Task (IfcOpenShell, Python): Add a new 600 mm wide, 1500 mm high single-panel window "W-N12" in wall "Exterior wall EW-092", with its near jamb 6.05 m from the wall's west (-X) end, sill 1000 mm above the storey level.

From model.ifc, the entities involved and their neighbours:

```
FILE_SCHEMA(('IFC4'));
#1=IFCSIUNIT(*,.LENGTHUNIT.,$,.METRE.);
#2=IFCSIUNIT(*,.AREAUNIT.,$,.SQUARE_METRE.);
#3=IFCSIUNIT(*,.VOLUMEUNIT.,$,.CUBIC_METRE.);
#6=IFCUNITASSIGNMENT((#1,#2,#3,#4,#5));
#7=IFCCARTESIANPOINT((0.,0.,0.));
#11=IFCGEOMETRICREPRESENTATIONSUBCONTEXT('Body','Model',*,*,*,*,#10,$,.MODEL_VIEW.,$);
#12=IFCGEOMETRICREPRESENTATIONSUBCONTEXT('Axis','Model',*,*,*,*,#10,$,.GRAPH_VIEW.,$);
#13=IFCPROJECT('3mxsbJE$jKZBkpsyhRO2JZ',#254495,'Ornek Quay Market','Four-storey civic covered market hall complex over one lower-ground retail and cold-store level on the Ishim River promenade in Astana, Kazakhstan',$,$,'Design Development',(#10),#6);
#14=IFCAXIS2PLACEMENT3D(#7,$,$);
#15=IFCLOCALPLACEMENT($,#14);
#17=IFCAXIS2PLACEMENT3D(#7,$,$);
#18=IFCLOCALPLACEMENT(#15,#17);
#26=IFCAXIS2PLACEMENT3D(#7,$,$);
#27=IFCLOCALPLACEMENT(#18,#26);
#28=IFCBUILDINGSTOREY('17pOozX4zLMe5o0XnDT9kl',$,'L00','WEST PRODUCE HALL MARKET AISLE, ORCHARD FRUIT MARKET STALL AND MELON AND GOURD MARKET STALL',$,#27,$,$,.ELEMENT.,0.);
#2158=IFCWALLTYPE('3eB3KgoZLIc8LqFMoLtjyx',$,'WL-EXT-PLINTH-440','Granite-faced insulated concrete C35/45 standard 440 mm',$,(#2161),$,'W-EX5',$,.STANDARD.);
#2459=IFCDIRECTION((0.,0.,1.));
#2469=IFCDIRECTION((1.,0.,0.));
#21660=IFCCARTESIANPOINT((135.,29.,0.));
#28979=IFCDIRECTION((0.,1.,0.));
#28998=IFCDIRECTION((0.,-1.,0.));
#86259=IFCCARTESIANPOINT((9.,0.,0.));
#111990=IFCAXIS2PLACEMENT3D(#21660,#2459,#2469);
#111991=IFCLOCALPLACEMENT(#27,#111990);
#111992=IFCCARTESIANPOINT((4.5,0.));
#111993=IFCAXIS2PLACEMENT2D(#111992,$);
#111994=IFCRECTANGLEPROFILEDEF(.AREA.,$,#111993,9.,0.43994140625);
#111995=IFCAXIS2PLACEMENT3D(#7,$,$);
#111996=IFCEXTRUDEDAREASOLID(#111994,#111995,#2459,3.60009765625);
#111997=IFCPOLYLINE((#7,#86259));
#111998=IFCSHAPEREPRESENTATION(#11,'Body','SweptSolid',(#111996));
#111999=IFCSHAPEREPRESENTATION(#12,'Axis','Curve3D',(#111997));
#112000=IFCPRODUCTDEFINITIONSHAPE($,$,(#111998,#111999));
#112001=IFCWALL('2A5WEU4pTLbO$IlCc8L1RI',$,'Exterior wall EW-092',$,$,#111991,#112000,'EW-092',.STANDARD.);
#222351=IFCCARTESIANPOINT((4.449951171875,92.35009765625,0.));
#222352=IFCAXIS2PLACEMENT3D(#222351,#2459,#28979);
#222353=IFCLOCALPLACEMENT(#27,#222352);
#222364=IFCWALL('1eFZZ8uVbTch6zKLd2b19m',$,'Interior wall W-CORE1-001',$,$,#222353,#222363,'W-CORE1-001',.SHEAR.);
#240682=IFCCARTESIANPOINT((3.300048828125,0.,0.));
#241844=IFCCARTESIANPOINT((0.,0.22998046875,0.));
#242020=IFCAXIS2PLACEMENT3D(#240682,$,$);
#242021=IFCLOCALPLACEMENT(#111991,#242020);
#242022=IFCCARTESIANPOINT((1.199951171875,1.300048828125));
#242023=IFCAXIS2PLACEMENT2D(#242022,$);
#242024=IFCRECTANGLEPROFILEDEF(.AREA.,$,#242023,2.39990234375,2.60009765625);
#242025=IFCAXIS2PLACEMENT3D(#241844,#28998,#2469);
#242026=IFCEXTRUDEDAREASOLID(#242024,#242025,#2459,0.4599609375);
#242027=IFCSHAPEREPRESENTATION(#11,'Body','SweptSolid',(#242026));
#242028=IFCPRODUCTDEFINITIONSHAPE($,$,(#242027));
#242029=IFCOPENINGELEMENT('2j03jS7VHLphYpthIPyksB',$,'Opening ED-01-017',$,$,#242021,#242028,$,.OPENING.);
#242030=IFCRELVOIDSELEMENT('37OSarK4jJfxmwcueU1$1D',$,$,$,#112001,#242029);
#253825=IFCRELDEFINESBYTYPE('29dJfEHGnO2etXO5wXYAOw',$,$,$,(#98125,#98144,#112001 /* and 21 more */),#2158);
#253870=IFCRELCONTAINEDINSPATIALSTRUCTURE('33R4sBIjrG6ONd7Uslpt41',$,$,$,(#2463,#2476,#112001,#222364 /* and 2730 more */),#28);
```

```python
import numpy as np
import ifcopenshell
import ifcopenshell.api.feature
import ifcopenshell.api.geometry
import ifcopenshell.api.root
import ifcopenshell.api.spatial
import ifcopenshell.geom
import ifcopenshell.util.element
import ifcopenshell.util.placement
import ifcopenshell.util.representation
import ifcopenshell.util.shape
import ifcopenshell.util.unit

model = ifcopenshell.open("model.ifc")
unit_scale = ifcopenshell.util.unit.calculate_unit_scale(model)
settings = ifcopenshell.geom.settings()


def volume(element):
    """Net volume in cubic metres, openings subtracted."""
    shape = ifcopenshell.geom.create_shape(settings, element)
    return ifcopenshell.util.shape.get_volume(shape.geometry)


wall = model.by_guid("2A5WEU4pTLbO$IlCc8L1RI")
storey = ifcopenshell.util.element.get_container(wall, ifc_class="IfcBuildingStorey")
context = ifcopenshell.util.representation.get_context(model, "Model", "Body", "MODEL_VIEW")
before = volume(wall)

width, height, from_end, sill = 0.6, 1.5, 6.05, 1  # metres

# The wall runs along its own X axis, and the end named is its -X end.
wall_shape = ifcopenshell.geom.create_shape(settings, wall)
x, y, z = ifcopenshell.util.shape.get_vertices(wall_shape.geometry).T
start = x.min() + from_end
face, thickness = float(y.min()), float(y.max() - y.min())
wall_matrix = ifcopenshell.util.placement.get_local_placement(wall.ObjectPlacement)
level = ifcopenshell.util.placement.get_local_placement(storey.ObjectPlacement)[2, 3]


def in_wall(x, y):
    """Placement at x, y metres in the wall's axes, at sill height."""
    matrix = wall_matrix.copy()
    matrix[:, 3] = wall_matrix @ np.array([x / unit_scale, y / unit_scale, 0.0, 1.0])
    matrix[2, 3] = level + sill / unit_scale
    return matrix


# Opening: a box that overshoots both wall faces by 50 mm.
opening = ifcopenshell.api.root.create_entity(model, ifc_class="IfcOpeningElement", predefined_type="OPENING")
box = ifcopenshell.api.geometry.add_wall_representation(
    model, context=context, length=width, height=height, thickness=thickness + 0.1
)
ifcopenshell.api.geometry.assign_representation(model, product=opening, representation=box)
ifcopenshell.api.geometry.edit_object_placement(model, product=opening, matrix=in_wall(start, face - 0.05), is_si=False)
ifcopenshell.api.feature.add_feature(model, feature=opening, element=wall)

window = ifcopenshell.api.root.create_entity(model, ifc_class="IfcWindow", name="W-N12", predefined_type="WINDOW")
window.OverallWidth, window.OverallHeight = width / unit_scale, height / unit_scale
window.PartitioningType = "SINGLE_PANEL"
body = ifcopenshell.api.geometry.add_window_representation(
    model,
    context=context,
    overall_width=window.OverallWidth,
    overall_height=window.OverallHeight,
    partition_type="SINGLE_PANEL",
)
ifcopenshell.api.geometry.assign_representation(model, product=window, representation=body)
ifcopenshell.api.spatial.assign_container(model, products=[window], relating_structure=storey)
ifcopenshell.api.feature.add_filling(model, opening=opening, element=window)

# Centre the window in the wall's thickness.
ifcopenshell.api.geometry.edit_object_placement(model, product=window, matrix=in_wall(start, face), is_si=False)
window_shape = ifcopenshell.geom.create_shape(settings, window)
depth = ifcopenshell.util.shape.get_vertices(window_shape.geometry)[:, 1]
offset = face + thickness / 2 - (depth.min() + depth.max()) / 2
ifcopenshell.api.geometry.edit_object_placement(model, product=window, matrix=in_wall(start, offset), is_si=False)

after = volume(wall)

print(f"wall volume {before:.3f} -> {after:.3f} m3")

model.write("model-out.ifc")
```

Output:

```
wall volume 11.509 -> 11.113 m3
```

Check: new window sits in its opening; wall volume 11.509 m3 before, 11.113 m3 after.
